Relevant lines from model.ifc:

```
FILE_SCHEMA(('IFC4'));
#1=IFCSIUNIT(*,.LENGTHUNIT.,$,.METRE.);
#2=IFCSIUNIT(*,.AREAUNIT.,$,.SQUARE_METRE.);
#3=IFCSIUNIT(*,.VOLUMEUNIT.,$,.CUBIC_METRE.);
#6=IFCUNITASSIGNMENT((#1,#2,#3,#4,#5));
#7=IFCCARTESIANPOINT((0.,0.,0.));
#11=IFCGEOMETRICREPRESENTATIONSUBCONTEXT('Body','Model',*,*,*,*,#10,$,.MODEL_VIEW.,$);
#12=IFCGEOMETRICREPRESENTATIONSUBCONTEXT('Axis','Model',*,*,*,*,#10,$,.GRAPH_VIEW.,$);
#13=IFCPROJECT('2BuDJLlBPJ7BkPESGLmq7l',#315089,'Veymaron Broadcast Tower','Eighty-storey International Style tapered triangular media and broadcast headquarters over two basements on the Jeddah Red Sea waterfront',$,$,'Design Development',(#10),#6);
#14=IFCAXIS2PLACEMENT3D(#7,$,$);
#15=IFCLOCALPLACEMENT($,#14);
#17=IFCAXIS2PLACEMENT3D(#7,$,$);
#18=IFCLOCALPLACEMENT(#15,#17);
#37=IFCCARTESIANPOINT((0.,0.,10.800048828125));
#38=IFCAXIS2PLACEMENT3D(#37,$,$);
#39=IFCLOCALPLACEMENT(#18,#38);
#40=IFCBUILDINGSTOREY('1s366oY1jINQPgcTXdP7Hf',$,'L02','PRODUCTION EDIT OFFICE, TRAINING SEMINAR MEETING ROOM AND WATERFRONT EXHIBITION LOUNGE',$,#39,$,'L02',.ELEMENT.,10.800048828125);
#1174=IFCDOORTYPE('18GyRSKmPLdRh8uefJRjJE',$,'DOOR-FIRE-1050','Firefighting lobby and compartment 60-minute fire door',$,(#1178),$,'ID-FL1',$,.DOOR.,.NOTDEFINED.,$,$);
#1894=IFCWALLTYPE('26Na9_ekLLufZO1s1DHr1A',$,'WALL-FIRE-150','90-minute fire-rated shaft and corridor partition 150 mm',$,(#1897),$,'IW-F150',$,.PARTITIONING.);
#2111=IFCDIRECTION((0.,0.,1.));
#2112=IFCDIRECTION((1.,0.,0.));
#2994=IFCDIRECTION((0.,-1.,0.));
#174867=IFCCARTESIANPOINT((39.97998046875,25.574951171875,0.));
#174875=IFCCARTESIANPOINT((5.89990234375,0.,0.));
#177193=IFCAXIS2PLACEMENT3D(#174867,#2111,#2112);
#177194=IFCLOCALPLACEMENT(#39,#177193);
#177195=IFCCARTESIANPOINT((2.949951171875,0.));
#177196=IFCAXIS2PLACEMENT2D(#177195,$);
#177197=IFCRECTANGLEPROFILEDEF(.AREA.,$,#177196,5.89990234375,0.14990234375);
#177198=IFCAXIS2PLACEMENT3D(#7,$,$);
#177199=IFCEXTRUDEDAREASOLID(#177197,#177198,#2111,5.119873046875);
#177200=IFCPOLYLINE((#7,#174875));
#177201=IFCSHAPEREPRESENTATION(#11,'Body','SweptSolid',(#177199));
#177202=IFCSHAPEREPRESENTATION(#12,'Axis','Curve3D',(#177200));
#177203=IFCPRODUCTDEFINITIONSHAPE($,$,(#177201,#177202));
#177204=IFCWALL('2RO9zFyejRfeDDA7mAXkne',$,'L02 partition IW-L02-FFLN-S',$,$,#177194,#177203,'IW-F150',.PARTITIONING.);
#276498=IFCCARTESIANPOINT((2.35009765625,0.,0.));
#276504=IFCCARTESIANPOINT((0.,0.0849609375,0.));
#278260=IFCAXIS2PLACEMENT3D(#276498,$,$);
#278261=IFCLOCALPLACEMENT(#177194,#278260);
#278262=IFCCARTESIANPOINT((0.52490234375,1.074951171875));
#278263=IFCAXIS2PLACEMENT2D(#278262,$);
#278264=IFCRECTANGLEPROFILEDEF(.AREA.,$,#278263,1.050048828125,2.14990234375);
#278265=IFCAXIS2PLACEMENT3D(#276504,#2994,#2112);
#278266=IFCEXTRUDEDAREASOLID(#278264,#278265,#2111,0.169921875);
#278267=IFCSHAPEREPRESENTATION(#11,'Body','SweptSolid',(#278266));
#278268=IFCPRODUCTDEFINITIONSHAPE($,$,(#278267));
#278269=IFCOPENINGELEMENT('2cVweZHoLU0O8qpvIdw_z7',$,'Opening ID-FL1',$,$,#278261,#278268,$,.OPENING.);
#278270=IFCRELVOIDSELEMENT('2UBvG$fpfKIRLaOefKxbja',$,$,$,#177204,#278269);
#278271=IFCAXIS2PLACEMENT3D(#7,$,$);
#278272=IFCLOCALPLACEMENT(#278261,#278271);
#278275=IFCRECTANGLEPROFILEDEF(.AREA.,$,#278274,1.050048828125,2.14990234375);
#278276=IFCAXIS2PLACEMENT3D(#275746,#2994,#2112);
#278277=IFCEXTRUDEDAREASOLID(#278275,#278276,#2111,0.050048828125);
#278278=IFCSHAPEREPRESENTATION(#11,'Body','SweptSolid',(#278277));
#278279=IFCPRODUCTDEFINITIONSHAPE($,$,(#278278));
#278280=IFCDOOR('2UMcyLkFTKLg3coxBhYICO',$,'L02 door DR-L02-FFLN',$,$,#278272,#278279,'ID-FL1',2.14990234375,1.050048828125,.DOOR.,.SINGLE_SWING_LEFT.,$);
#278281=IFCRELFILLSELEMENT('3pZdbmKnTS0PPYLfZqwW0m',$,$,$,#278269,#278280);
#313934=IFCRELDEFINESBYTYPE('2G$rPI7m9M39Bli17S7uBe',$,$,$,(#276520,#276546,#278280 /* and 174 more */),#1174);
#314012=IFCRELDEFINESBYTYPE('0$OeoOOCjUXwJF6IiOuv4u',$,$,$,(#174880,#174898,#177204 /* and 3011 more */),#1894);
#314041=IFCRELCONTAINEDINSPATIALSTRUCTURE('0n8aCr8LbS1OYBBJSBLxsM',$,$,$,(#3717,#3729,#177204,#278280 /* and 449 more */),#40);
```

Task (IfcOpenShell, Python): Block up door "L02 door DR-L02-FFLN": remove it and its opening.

```python
import ifcopenshell
import ifcopenshell.api.feature
import ifcopenshell.api.root
import ifcopenshell.geom
import ifcopenshell.util.shape

model = ifcopenshell.open("model.ifc")
settings = ifcopenshell.geom.settings()


def volume(element):
    """Net volume in cubic metres, openings subtracted."""
    shape = ifcopenshell.geom.create_shape(settings, element)
    return ifcopenshell.util.shape.get_volume(shape.geometry)


door = model.by_guid("2UMcyLkFTKLg3coxBhYICO")
opening = door.FillsVoids[0].RelatingOpeningElement
wall = opening.VoidsElements[0].RelatingBuildingElement
before = volume(wall)

ifcopenshell.api.root.remove_product(model, product=door)
ifcopenshell.api.feature.remove_feature(model, feature=opening)

after = volume(wall)

print(f"wall volume {before:.3f} -> {after:.3f} m3")

model.write("model_v2.ifc")
```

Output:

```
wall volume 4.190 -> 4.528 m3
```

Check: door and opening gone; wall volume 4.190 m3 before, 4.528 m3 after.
